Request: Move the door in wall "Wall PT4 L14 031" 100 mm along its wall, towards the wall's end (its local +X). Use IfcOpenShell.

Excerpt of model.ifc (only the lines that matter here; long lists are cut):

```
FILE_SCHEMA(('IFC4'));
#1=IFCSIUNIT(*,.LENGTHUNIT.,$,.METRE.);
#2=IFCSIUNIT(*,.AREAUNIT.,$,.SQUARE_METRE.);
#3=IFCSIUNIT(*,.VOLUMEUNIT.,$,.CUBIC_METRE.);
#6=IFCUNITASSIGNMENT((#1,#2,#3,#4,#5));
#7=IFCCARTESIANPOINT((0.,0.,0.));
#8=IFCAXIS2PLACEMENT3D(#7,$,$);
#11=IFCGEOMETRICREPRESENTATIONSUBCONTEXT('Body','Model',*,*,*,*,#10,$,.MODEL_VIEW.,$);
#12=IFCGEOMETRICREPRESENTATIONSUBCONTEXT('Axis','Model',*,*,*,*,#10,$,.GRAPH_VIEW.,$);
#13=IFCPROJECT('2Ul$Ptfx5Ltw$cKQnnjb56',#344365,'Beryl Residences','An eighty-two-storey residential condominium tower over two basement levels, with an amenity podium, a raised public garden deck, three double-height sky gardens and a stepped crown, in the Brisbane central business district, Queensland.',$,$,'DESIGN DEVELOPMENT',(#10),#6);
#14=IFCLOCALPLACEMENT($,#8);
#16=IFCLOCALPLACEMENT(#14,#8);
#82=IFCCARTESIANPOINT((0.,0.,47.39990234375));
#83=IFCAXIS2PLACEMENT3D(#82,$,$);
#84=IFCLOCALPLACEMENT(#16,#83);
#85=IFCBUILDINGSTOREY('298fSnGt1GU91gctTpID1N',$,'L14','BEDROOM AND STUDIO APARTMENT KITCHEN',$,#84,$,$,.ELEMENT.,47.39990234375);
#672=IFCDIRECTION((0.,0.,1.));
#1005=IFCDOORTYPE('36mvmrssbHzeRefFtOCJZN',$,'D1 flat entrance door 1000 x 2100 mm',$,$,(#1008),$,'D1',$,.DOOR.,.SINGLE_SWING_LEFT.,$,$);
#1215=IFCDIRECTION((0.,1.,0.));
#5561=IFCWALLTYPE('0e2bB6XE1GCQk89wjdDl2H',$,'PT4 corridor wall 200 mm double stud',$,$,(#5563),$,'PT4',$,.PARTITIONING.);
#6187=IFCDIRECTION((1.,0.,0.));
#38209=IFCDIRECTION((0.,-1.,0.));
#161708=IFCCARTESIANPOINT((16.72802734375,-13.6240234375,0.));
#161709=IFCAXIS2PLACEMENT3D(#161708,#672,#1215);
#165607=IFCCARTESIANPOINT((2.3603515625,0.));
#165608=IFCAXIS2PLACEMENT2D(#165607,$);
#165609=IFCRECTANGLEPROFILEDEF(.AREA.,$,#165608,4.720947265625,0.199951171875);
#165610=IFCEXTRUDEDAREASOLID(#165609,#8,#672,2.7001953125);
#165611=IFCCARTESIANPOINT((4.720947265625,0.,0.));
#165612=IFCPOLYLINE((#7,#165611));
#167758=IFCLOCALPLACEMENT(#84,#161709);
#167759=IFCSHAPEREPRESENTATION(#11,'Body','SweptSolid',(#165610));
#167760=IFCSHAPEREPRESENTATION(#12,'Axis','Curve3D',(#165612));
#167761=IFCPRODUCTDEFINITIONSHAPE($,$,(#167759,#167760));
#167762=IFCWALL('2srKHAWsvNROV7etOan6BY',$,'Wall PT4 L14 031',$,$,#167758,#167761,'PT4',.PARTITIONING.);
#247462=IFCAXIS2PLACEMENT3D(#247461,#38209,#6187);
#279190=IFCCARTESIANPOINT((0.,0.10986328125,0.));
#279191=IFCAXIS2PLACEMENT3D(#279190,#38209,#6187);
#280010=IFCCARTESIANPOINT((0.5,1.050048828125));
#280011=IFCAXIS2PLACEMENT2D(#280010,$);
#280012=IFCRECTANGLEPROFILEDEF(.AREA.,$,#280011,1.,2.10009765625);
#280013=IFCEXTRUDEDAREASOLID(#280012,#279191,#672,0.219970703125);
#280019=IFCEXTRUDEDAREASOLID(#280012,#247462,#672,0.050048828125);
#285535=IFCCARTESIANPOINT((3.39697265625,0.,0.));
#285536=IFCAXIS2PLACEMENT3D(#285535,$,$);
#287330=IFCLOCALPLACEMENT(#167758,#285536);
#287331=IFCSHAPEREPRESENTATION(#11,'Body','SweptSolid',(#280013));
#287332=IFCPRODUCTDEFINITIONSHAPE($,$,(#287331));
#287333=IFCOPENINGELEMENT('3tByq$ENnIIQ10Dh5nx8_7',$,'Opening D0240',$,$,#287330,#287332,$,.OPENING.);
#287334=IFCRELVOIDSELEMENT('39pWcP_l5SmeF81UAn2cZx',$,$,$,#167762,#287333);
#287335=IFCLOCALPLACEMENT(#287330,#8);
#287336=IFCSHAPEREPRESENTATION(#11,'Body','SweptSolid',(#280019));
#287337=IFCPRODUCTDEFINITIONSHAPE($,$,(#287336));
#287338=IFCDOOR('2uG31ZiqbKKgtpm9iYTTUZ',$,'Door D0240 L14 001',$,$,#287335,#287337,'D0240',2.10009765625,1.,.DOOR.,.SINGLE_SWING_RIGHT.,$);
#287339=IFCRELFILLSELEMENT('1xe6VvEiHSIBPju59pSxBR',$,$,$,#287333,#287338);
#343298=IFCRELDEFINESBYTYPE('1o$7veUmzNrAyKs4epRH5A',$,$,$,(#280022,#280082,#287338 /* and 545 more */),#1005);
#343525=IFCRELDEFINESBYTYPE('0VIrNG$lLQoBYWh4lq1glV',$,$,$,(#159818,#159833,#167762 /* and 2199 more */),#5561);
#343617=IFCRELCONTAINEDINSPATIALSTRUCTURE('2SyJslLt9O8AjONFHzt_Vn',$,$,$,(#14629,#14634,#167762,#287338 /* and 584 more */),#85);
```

```python
import ifcopenshell
import ifcopenshell.api.geometry
import ifcopenshell.util.placement
import ifcopenshell.util.unit

model = ifcopenshell.open("model.ifc")
unit_scale = ifcopenshell.util.unit.calculate_unit_scale(model)

door = model.by_guid("2uG31ZiqbKKgtpm9iYTTUZ")
opening = door.FillsVoids[0].RelatingOpeningElement
wall = opening.VoidsElements[0].RelatingBuildingElement

wall_matrix = ifcopenshell.util.placement.get_local_placement(wall.ObjectPlacement)
shift = wall_matrix[:3, 0] * 0.1 / unit_scale
before = ifcopenshell.util.placement.get_local_placement(door.ObjectPlacement)[:3, 3].copy()

# The door is placed relative to its opening, so it follows when the opening moves.
matrix = ifcopenshell.util.placement.get_local_placement(opening.ObjectPlacement)
matrix[:3, 3] += shift
ifcopenshell.api.geometry.edit_object_placement(
    model, product=opening, matrix=matrix, is_si=False, should_transform_children=True
)

after = ifcopenshell.util.placement.get_local_placement(door.ObjectPlacement)[:3, 3]
print("door moved by", (after - before).round(3) + 0.0)

model.write("model-out.ifc")
```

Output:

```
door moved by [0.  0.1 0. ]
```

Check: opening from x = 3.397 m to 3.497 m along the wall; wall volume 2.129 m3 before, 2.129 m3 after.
